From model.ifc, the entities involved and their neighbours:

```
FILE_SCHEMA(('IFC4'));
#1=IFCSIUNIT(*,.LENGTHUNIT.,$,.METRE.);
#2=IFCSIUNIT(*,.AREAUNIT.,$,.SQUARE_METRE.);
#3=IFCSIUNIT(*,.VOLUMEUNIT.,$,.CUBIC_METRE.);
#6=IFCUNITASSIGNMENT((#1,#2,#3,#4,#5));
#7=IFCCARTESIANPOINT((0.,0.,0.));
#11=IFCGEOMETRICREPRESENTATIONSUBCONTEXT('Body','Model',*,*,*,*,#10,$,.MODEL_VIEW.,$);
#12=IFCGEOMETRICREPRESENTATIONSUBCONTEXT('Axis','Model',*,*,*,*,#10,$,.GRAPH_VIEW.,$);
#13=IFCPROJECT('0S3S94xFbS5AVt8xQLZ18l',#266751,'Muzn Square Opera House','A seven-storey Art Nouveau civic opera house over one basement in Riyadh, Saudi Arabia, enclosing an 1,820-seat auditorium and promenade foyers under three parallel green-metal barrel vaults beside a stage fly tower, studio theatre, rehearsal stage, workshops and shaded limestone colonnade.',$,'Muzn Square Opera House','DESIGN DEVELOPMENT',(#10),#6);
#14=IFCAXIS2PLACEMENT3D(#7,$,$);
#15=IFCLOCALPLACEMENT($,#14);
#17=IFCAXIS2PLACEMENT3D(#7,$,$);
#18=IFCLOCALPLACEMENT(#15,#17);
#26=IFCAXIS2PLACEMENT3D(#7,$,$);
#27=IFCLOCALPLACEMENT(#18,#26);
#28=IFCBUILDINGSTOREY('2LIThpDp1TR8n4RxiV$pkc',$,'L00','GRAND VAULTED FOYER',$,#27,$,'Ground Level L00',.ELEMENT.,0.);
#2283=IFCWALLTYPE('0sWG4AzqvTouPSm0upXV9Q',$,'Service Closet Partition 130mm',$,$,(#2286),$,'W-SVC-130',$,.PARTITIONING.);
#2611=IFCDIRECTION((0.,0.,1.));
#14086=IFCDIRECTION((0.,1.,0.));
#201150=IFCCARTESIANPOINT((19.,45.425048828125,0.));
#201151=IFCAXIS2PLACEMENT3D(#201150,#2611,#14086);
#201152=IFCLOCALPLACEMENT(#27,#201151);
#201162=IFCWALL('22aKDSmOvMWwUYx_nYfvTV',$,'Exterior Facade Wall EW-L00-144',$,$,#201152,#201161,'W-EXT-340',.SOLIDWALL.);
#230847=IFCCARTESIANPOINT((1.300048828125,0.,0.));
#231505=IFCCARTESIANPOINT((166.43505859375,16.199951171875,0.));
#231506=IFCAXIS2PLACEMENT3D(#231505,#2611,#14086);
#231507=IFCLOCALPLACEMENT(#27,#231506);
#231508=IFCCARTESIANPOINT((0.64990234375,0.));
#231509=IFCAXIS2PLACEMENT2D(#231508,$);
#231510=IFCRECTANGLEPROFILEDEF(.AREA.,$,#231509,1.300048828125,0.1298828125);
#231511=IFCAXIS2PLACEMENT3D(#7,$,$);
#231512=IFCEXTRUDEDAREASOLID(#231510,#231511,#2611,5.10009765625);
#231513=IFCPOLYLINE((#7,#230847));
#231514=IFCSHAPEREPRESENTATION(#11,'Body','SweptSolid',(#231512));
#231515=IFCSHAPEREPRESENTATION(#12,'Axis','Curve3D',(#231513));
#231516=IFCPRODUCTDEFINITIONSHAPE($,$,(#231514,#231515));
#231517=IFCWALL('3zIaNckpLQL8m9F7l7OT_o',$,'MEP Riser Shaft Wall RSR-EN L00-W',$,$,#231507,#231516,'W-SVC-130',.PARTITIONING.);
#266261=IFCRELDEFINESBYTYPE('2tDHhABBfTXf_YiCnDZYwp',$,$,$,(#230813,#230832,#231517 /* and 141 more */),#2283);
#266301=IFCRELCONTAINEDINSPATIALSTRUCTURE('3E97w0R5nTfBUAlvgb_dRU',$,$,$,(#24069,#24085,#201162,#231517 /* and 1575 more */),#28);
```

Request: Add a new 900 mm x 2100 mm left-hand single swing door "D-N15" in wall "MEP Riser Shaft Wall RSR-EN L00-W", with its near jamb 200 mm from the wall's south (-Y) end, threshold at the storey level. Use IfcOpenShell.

```python
import numpy as np
import ifcopenshell
import ifcopenshell.api.feature
import ifcopenshell.api.geometry
import ifcopenshell.api.root
import ifcopenshell.api.spatial
import ifcopenshell.geom
import ifcopenshell.util.element
import ifcopenshell.util.placement
import ifcopenshell.util.representation
import ifcopenshell.util.shape
import ifcopenshell.util.unit

model = ifcopenshell.open("model.ifc")
unit_scale = ifcopenshell.util.unit.calculate_unit_scale(model)
settings = ifcopenshell.geom.settings()


def volume(element):
    """Net volume in cubic metres, openings subtracted."""
    shape = ifcopenshell.geom.create_shape(settings, element)
    return ifcopenshell.util.shape.get_volume(shape.geometry)


wall = model.by_guid("3zIaNckpLQL8m9F7l7OT_o")
storey = ifcopenshell.util.element.get_container(wall, ifc_class="IfcBuildingStorey")
context = ifcopenshell.util.representation.get_context(model, "Model", "Body", "MODEL_VIEW")
before = volume(wall)

width, height, from_end, sill = 0.9, 2.1, 0.2, 0.0  # metres

# The wall runs along its own X axis, and the end named is its -X end.
wall_shape = ifcopenshell.geom.create_shape(settings, wall)
x, y, z = ifcopenshell.util.shape.get_vertices(wall_shape.geometry).T
start = x.min() + from_end
face, thickness = float(y.min()), float(y.max() - y.min())
wall_matrix = ifcopenshell.util.placement.get_local_placement(wall.ObjectPlacement)
level = ifcopenshell.util.placement.get_local_placement(storey.ObjectPlacement)[2, 3]


def in_wall(x, y):
    """Placement at x, y metres in the wall's axes, at sill height."""
    matrix = wall_matrix.copy()
    matrix[:, 3] = wall_matrix @ np.array([x / unit_scale, y / unit_scale, 0.0, 1.0])
    matrix[2, 3] = level + sill / unit_scale
    return matrix


# Opening: a box that overshoots both wall faces by 50 mm.
opening = ifcopenshell.api.root.create_entity(model, ifc_class="IfcOpeningElement", predefined_type="OPENING")
box = ifcopenshell.api.geometry.add_wall_representation(
    model, context=context, length=width, height=height, thickness=thickness + 0.1
)
ifcopenshell.api.geometry.assign_representation(model, product=opening, representation=box)
ifcopenshell.api.geometry.edit_object_placement(model, product=opening, matrix=in_wall(start, face - 0.05), is_si=False)
ifcopenshell.api.feature.add_feature(model, feature=opening, element=wall)

door = ifcopenshell.api.root.create_entity(model, ifc_class="IfcDoor", name="D-N15", predefined_type="DOOR")
door.OverallWidth, door.OverallHeight = width / unit_scale, height / unit_scale
door.OperationType = "SINGLE_SWING_LEFT"
body = ifcopenshell.api.geometry.add_door_representation(
    model,
    context=context,
    overall_width=door.OverallWidth,
    overall_height=door.OverallHeight,
    operation_type="SINGLE_SWING_LEFT",
    lining_properties={"LiningDepth": thickness / unit_scale, "ThresholdDepth": thickness / unit_scale},
)
ifcopenshell.api.geometry.assign_representation(model, product=door, representation=body)
ifcopenshell.api.spatial.assign_container(model, products=[door], relating_structure=storey)
ifcopenshell.api.feature.add_filling(model, opening=opening, element=door)

# The lining spans the wall, so the door starts at the wall face.
ifcopenshell.api.geometry.edit_object_placement(model, product=door, matrix=in_wall(start, face), is_si=False)

after = volume(wall)

print(f"wall volume {before:.3f} -> {after:.3f} m3")

model.write("model_edited.ifc")
```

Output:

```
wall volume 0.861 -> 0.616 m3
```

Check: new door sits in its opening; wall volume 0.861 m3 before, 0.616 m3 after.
